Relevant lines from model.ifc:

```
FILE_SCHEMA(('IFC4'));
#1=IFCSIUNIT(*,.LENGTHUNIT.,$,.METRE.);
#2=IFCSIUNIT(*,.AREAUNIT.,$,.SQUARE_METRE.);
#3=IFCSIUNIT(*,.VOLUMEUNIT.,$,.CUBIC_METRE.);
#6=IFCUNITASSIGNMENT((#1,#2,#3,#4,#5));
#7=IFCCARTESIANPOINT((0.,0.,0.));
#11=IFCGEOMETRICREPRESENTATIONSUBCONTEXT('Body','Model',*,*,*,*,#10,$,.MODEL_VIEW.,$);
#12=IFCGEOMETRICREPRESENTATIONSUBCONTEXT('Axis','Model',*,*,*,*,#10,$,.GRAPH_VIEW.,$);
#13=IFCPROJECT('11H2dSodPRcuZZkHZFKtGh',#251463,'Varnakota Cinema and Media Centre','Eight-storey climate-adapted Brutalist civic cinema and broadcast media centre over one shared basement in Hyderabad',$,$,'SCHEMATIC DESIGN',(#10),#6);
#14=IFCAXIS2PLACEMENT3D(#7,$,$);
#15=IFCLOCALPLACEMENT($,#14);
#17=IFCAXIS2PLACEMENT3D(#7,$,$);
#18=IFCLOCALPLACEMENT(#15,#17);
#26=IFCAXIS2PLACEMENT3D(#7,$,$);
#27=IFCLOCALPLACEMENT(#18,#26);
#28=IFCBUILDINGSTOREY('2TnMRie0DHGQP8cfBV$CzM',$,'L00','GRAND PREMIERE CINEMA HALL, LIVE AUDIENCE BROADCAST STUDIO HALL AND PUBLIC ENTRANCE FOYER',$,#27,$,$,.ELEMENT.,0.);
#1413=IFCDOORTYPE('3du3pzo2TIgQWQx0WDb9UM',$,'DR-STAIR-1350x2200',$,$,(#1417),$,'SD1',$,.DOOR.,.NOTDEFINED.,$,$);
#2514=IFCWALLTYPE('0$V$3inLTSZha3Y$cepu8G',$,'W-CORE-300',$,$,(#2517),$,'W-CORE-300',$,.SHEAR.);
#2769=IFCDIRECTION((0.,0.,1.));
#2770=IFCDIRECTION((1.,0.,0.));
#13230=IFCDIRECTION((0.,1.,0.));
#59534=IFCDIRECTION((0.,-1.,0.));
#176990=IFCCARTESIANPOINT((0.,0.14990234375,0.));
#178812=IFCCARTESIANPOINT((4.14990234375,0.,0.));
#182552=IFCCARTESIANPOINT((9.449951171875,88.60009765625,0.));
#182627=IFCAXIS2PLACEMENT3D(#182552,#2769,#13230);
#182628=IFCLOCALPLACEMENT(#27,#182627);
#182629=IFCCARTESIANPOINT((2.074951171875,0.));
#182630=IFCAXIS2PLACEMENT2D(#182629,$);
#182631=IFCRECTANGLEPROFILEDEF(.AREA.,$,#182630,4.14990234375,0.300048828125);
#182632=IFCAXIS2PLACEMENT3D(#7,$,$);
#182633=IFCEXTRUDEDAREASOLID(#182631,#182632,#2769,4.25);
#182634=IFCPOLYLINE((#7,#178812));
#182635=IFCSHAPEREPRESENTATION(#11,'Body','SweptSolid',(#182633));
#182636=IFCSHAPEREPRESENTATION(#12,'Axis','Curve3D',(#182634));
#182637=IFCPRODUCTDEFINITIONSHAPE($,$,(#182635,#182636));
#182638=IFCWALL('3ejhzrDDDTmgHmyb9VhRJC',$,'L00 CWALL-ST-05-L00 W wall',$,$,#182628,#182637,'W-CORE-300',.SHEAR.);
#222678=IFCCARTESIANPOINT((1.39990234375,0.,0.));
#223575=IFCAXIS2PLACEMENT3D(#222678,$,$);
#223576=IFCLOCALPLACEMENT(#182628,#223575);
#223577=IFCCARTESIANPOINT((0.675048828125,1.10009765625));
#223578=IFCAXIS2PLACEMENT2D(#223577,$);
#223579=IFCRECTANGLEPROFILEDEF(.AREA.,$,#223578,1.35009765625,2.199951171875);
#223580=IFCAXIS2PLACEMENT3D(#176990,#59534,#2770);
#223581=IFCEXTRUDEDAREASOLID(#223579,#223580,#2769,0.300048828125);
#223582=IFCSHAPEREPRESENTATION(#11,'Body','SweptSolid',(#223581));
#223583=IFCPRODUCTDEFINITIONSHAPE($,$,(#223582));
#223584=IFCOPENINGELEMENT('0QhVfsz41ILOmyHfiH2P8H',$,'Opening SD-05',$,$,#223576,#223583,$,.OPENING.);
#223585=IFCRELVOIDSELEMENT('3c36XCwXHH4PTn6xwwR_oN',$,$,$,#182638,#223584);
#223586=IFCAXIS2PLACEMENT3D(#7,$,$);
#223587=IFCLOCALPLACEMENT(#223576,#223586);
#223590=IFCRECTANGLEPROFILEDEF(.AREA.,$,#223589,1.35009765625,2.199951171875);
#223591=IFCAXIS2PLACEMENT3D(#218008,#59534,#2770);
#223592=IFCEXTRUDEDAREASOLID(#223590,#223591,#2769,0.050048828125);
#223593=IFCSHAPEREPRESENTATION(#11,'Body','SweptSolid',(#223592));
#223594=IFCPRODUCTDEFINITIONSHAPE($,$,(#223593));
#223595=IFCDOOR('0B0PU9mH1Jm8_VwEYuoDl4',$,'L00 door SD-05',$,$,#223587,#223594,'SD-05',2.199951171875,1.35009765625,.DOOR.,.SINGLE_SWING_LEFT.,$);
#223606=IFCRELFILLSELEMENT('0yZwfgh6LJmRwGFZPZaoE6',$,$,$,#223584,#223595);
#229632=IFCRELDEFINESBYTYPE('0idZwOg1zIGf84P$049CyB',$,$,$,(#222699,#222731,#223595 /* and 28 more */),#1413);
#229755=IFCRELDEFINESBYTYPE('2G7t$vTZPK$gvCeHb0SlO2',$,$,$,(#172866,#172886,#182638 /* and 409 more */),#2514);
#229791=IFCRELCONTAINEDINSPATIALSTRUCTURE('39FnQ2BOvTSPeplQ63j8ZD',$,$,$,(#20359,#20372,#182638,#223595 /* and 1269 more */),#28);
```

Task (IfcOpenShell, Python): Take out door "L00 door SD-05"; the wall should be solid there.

```python
import ifcopenshell
import ifcopenshell.api.feature
import ifcopenshell.api.root
import ifcopenshell.geom
import ifcopenshell.util.shape

model = ifcopenshell.open("model.ifc")
settings = ifcopenshell.geom.settings()


def volume(element):
    """Net volume in cubic metres, openings subtracted."""
    shape = ifcopenshell.geom.create_shape(settings, element)
    return ifcopenshell.util.shape.get_volume(shape.geometry)


door = model.by_guid("0B0PU9mH1Jm8_VwEYuoDl4")
opening = door.FillsVoids[0].RelatingOpeningElement
wall = opening.VoidsElements[0].RelatingBuildingElement
before = volume(wall)

ifcopenshell.api.root.remove_product(model, product=door)
ifcopenshell.api.feature.remove_feature(model, feature=opening)

after = volume(wall)

print(f"wall volume {before:.3f} -> {after:.3f} m3")

model.write("model_updated.ifc")
```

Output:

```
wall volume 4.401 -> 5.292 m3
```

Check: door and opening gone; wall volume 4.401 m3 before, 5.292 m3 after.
